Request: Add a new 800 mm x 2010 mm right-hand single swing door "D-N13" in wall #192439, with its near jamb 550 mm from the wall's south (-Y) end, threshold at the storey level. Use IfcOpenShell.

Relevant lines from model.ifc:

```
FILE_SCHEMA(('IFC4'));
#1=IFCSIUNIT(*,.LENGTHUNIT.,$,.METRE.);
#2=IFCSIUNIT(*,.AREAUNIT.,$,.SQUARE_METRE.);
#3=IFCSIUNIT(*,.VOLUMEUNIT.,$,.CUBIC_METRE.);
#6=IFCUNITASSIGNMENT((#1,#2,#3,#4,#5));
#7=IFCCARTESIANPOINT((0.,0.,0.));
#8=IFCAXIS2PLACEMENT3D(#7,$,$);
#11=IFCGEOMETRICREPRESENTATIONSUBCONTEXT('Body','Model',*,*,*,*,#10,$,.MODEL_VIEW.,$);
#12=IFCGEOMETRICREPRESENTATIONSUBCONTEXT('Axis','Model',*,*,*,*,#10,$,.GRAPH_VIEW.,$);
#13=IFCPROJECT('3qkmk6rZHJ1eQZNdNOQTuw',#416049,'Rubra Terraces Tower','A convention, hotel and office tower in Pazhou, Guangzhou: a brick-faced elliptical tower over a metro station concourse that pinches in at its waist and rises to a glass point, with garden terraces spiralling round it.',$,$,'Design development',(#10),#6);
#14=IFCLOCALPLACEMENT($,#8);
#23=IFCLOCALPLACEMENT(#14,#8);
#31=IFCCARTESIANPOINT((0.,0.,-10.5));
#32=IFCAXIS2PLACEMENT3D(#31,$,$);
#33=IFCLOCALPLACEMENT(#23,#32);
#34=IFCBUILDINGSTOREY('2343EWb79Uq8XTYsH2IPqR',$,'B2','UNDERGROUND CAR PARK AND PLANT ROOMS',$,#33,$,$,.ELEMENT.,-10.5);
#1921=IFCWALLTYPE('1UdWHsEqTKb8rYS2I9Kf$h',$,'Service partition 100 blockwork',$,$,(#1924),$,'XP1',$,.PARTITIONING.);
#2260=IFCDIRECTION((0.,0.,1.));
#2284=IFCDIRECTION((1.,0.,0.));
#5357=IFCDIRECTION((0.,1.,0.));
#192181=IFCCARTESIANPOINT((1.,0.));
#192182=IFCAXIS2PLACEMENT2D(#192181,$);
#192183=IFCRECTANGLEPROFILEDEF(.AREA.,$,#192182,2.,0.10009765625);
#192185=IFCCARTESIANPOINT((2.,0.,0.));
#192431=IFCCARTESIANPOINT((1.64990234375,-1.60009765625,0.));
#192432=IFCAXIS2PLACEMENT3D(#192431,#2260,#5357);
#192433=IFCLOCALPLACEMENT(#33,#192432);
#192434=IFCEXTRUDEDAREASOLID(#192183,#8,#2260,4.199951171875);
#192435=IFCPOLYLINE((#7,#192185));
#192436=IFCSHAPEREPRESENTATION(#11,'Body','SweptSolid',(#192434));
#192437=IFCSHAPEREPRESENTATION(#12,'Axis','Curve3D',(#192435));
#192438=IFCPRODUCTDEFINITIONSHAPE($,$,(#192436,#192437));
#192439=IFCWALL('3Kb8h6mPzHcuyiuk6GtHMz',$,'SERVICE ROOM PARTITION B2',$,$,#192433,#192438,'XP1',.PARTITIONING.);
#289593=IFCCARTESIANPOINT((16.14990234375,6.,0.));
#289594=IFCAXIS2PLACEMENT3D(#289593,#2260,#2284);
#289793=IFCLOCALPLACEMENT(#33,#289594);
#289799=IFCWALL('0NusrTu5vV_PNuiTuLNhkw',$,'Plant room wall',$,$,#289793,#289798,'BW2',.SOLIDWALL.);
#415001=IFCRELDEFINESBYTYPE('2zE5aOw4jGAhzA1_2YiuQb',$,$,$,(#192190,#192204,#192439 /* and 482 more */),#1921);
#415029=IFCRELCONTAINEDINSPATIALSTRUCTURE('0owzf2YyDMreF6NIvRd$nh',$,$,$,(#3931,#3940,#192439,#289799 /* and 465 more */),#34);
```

```python
import numpy as np
import ifcopenshell
import ifcopenshell.api.feature
import ifcopenshell.api.geometry
import ifcopenshell.api.root
import ifcopenshell.api.spatial
import ifcopenshell.geom
import ifcopenshell.util.element
import ifcopenshell.util.placement
import ifcopenshell.util.representation
import ifcopenshell.util.shape
import ifcopenshell.util.unit

model = ifcopenshell.open("model.ifc")
unit_scale = ifcopenshell.util.unit.calculate_unit_scale(model)
settings = ifcopenshell.geom.settings()


def volume(element):
    """Net volume in cubic metres, openings subtracted."""
    shape = ifcopenshell.geom.create_shape(settings, element)
    return ifcopenshell.util.shape.get_volume(shape.geometry)


wall = model.by_guid("3Kb8h6mPzHcuyiuk6GtHMz")
storey = ifcopenshell.util.element.get_container(wall, ifc_class="IfcBuildingStorey")
context = ifcopenshell.util.representation.get_context(model, "Model", "Body", "MODEL_VIEW")
before = volume(wall)

width, height, from_end, sill = 0.8, 2.01, 0.55, 0.0  # metres

# The wall runs along its own X axis, and the end named is its -X end.
wall_shape = ifcopenshell.geom.create_shape(settings, wall)
x, y, z = ifcopenshell.util.shape.get_vertices(wall_shape.geometry).T
start = x.min() + from_end
face, thickness = float(y.min()), float(y.max() - y.min())
wall_matrix = ifcopenshell.util.placement.get_local_placement(wall.ObjectPlacement)
level = ifcopenshell.util.placement.get_local_placement(storey.ObjectPlacement)[2, 3]


def in_wall(x, y):
    """Placement at x, y metres in the wall's axes, at sill height."""
    matrix = wall_matrix.copy()
    matrix[:, 3] = wall_matrix @ np.array([x / unit_scale, y / unit_scale, 0.0, 1.0])
    matrix[2, 3] = level + sill / unit_scale
    return matrix


# Opening: a box that overshoots both wall faces by 50 mm.
opening = ifcopenshell.api.root.create_entity(model, ifc_class="IfcOpeningElement", predefined_type="OPENING")
box = ifcopenshell.api.geometry.add_wall_representation(
    model, context=context, length=width, height=height, thickness=thickness + 0.1
)
ifcopenshell.api.geometry.assign_representation(model, product=opening, representation=box)
ifcopenshell.api.geometry.edit_object_placement(model, product=opening, matrix=in_wall(start, face - 0.05), is_si=False)
ifcopenshell.api.feature.add_feature(model, feature=opening, element=wall)

door = ifcopenshell.api.root.create_entity(model, ifc_class="IfcDoor", name="D-N13", predefined_type="DOOR")
door.OverallWidth, door.OverallHeight = width / unit_scale, height / unit_scale
door.OperationType = "SINGLE_SWING_RIGHT"
body = ifcopenshell.api.geometry.add_door_representation(
    model,
    context=context,
    overall_width=door.OverallWidth,
    overall_height=door.OverallHeight,
    operation_type="SINGLE_SWING_RIGHT",
    lining_properties={"LiningDepth": thickness / unit_scale, "ThresholdDepth": thickness / unit_scale},
)
ifcopenshell.api.geometry.assign_representation(model, product=door, representation=body)
ifcopenshell.api.spatial.assign_container(model, products=[door], relating_structure=storey)
ifcopenshell.api.feature.add_filling(model, opening=opening, element=door)

# The lining spans the wall, so the door starts at the wall face.
ifcopenshell.api.geometry.edit_object_placement(model, product=door, matrix=in_wall(start, face), is_si=False)

after = volume(wall)

print(f"wall volume {before:.3f} -> {after:.3f} m3")

model.write("model_v2.ifc")
```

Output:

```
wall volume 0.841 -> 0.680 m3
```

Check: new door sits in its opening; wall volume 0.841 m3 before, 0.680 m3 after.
